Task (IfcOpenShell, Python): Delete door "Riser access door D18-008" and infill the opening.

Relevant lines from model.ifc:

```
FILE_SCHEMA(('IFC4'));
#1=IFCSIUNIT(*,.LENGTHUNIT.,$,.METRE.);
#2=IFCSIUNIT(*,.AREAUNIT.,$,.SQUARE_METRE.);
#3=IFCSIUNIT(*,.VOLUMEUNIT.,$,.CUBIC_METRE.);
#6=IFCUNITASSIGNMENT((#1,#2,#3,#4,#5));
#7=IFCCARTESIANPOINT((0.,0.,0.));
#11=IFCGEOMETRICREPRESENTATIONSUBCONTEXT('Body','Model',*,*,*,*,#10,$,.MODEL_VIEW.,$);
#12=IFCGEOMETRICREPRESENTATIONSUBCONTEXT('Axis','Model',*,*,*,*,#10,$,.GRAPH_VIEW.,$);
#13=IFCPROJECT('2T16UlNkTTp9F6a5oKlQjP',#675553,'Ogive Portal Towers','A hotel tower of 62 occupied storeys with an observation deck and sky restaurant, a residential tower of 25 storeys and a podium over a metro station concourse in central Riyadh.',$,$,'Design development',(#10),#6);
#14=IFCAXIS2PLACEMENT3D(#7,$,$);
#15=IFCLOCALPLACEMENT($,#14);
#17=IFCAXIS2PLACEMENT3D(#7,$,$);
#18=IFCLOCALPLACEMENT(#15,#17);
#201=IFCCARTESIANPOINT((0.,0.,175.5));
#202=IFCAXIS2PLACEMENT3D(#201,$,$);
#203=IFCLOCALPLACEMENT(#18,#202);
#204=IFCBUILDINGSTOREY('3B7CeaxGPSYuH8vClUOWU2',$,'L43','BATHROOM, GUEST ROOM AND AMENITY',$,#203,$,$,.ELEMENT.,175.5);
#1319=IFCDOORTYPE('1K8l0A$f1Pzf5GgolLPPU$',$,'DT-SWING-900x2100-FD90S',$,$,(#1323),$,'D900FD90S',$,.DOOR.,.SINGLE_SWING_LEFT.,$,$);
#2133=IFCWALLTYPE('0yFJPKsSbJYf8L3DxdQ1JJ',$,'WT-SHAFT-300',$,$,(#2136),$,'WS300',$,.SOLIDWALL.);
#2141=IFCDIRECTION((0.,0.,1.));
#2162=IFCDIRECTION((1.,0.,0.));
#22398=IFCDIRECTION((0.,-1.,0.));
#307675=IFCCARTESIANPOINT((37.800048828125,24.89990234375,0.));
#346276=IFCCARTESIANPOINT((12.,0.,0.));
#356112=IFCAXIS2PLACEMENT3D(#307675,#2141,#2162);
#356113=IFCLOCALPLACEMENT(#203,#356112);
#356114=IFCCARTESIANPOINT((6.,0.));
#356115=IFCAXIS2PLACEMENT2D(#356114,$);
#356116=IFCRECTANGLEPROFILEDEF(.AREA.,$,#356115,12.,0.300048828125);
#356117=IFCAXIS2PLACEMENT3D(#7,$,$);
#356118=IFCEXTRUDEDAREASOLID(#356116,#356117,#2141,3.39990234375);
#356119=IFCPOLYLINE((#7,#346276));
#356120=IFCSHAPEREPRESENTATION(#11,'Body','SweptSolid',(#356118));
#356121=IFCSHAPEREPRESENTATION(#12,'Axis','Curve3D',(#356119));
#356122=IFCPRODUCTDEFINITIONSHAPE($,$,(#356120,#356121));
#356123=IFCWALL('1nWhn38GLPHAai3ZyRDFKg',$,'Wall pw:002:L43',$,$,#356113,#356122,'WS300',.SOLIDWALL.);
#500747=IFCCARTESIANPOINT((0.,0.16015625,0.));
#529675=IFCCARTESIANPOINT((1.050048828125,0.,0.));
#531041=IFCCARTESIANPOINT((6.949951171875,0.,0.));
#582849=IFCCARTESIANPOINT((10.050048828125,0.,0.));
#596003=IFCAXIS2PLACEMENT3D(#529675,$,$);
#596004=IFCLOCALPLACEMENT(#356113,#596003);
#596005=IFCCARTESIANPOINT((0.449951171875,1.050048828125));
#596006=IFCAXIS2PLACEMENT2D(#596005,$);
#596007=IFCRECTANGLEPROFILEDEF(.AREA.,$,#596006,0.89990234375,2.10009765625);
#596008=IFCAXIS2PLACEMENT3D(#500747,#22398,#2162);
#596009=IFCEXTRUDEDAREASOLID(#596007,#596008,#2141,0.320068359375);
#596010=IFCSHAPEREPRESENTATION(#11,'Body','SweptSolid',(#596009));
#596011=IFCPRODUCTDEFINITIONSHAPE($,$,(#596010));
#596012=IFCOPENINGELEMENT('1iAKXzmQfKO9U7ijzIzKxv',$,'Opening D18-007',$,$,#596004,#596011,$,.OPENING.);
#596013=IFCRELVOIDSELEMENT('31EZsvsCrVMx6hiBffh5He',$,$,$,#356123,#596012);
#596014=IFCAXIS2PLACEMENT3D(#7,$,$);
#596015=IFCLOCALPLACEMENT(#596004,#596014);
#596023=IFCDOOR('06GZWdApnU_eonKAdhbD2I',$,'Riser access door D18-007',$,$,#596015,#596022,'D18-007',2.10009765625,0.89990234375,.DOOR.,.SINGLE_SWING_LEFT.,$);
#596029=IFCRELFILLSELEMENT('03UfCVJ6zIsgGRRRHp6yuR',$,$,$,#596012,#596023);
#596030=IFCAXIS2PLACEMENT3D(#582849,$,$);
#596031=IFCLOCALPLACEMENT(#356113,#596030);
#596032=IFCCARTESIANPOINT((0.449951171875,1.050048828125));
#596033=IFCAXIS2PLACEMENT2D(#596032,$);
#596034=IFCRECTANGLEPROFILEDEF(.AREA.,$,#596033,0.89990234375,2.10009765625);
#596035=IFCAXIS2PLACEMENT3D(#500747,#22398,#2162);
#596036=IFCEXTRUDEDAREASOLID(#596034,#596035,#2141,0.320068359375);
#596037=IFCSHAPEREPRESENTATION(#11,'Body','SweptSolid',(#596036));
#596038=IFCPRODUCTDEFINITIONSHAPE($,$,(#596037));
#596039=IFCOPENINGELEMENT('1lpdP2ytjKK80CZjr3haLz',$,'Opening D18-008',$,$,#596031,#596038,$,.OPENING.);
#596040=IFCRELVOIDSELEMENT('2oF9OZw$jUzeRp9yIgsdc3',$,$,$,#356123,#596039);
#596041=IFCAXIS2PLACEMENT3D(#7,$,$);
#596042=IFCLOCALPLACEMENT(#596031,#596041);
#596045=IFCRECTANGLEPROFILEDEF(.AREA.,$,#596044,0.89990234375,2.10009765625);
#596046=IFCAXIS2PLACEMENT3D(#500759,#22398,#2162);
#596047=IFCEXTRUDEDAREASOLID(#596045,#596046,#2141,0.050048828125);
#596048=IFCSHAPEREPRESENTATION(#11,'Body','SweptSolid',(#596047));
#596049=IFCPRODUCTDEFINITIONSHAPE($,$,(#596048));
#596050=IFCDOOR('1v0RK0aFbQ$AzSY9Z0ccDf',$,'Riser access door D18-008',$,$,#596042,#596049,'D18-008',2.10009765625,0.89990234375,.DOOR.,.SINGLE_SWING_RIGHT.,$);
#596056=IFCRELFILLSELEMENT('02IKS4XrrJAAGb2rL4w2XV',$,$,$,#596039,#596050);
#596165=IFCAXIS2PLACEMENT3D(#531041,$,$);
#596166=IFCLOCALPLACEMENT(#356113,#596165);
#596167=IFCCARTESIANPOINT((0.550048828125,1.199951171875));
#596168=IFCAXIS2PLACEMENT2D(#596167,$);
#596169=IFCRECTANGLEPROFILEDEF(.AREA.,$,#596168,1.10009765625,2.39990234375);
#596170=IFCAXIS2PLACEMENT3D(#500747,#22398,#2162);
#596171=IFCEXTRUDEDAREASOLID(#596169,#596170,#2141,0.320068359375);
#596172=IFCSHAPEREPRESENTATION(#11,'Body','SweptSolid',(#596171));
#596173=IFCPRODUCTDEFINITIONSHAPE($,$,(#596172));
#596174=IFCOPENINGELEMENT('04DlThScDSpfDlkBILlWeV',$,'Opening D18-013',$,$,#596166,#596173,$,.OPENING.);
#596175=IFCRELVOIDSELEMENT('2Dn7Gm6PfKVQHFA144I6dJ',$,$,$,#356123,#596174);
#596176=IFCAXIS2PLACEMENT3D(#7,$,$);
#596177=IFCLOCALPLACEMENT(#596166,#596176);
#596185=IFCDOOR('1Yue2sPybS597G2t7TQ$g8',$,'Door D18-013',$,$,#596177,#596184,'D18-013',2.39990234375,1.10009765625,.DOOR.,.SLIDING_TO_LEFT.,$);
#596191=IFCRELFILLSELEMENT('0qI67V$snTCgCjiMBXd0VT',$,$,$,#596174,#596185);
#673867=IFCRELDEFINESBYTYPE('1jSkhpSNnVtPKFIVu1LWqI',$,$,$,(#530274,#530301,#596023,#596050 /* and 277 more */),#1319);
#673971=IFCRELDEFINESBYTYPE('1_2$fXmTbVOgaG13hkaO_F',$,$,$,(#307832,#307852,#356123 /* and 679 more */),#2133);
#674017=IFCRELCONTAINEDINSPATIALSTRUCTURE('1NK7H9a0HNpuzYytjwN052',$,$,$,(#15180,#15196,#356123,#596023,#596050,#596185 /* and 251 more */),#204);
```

```python
import ifcopenshell
import ifcopenshell.api.feature
import ifcopenshell.api.root
import ifcopenshell.geom
import ifcopenshell.util.shape

model = ifcopenshell.open("model.ifc")
settings = ifcopenshell.geom.settings()


def volume(element):
    """Net volume in cubic metres, openings subtracted."""
    shape = ifcopenshell.geom.create_shape(settings, element)
    return ifcopenshell.util.shape.get_volume(shape.geometry)


door = model.by_guid("1v0RK0aFbQ$AzSY9Z0ccDf")
opening = door.FillsVoids[0].RelatingOpeningElement
wall = opening.VoidsElements[0].RelatingBuildingElement
before = volume(wall)

ifcopenshell.api.root.remove_product(model, product=door)
ifcopenshell.api.feature.remove_feature(model, feature=opening)

after = volume(wall)

print(f"wall volume {before:.3f} -> {after:.3f} m3")

model.write("model-out.ifc")
```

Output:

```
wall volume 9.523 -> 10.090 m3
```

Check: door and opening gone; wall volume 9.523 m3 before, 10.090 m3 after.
